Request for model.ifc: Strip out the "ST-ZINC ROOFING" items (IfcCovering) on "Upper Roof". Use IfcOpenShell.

First a look at what the model holds.

```python
import ifcopenshell
import ifcopenshell.util.element

model = ifcopenshell.open("model.ifc")
print(model.schema)
storey = next(s for s in model.by_type("IfcBuildingStorey") if s.Name == "Upper Roof")
coverings = [e for e in ifcopenshell.util.element.get_decomposition(storey) if e.is_a("IfcCovering")]
seen = {}
for e in coverings:
    element_type = ifcopenshell.util.element.get_type(e)
    name = element_type.Name if element_type not in (None, e) else None
    seen[name] = seen.get(name, 0) + 1
for name, count in sorted(seen.items(), key=str):
    print(count, "x", name)
```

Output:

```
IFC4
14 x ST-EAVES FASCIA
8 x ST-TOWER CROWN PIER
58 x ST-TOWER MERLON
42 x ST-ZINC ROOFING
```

```python
import ifcopenshell
import ifcopenshell.api.root
import ifcopenshell.util.element

model = ifcopenshell.open("model.ifc")

storey = next(s for s in model.by_type("IfcBuildingStorey") if s.Name == "Upper Roof")
coverings = [e for e in ifcopenshell.util.element.get_decomposition(storey) if e.is_a("IfcCovering")]
targets = [e for e in coverings if (t := ifcopenshell.util.element.get_type(e)) not in (None, e) and t.Name == "ST-ZINC ROOFING"]

for e in targets:
    ifcopenshell.api.root.remove_product(model, product=e)
print(len(targets), "removed")

model.write("model-out.ifc")
```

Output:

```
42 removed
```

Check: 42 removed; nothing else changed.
